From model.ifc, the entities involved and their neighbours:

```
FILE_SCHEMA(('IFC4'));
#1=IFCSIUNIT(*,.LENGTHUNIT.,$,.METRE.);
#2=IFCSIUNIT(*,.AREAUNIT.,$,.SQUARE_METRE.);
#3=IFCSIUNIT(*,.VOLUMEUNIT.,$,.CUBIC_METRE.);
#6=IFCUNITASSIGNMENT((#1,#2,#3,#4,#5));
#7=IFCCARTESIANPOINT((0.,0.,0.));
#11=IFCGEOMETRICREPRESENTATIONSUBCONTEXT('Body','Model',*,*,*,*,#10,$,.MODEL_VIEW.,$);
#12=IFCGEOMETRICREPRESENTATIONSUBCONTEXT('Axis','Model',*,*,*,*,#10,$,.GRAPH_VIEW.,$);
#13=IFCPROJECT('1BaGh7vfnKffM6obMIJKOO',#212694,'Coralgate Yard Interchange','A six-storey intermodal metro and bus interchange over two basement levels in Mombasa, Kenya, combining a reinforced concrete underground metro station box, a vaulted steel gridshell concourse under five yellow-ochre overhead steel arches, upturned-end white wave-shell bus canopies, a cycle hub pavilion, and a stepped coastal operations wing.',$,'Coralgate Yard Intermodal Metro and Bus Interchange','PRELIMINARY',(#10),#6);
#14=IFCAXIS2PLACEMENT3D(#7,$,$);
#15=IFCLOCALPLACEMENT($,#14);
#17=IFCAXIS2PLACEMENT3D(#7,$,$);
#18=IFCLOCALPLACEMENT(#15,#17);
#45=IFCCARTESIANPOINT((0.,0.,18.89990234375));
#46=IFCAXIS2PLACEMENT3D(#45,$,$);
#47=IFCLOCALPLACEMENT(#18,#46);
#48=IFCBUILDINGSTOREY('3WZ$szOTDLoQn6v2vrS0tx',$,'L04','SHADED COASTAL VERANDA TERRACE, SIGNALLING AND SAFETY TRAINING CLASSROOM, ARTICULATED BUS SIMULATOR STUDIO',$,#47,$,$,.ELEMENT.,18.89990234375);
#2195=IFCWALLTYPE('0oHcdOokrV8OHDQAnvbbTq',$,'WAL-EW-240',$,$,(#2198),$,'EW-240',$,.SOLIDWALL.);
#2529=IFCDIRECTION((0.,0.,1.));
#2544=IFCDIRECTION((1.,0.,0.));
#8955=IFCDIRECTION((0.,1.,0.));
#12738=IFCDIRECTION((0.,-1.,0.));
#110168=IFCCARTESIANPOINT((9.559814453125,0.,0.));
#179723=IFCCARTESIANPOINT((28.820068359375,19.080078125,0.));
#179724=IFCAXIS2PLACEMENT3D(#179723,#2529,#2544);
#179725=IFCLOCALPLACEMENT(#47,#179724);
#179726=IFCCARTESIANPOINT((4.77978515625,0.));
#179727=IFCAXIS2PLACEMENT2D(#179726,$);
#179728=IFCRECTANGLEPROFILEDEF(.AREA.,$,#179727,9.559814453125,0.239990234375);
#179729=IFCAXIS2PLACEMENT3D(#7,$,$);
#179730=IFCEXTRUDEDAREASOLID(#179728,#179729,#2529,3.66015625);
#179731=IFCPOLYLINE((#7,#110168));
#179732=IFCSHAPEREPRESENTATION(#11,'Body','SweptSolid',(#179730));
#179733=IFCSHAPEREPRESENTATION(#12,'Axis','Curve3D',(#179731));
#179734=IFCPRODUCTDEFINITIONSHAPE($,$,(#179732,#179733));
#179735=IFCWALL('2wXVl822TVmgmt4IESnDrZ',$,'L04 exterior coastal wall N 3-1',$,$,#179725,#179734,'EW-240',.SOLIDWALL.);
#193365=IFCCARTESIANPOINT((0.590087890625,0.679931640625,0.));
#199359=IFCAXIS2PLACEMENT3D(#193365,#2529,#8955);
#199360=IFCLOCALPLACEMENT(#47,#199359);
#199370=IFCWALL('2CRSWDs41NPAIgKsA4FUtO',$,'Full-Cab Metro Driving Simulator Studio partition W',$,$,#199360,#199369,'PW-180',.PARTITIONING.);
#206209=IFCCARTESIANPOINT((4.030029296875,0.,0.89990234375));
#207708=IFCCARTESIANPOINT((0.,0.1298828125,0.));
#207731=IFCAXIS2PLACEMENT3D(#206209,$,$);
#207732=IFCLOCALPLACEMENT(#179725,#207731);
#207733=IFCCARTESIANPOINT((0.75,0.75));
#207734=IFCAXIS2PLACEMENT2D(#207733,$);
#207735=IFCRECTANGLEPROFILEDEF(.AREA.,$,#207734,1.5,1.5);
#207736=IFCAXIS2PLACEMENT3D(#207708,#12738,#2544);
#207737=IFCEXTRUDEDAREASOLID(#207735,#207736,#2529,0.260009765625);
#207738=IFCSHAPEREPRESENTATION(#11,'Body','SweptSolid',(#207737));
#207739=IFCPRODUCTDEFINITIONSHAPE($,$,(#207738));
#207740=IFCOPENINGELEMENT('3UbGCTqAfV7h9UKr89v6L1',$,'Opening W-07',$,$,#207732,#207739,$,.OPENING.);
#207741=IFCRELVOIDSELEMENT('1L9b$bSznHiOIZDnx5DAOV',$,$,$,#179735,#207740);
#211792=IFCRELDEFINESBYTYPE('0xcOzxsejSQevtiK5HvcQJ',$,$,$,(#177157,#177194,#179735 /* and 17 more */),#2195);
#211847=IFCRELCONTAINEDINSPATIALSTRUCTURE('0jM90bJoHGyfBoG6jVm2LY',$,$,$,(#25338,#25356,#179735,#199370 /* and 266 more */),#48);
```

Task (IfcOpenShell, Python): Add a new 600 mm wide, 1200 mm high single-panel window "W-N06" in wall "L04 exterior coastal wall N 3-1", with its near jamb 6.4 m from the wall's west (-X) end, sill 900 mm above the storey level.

```python
import numpy as np
import ifcopenshell
import ifcopenshell.api.feature
import ifcopenshell.api.geometry
import ifcopenshell.api.root
import ifcopenshell.api.spatial
import ifcopenshell.geom
import ifcopenshell.util.element
import ifcopenshell.util.placement
import ifcopenshell.util.representation
import ifcopenshell.util.shape
import ifcopenshell.util.unit

model = ifcopenshell.open("model.ifc")
unit_scale = ifcopenshell.util.unit.calculate_unit_scale(model)
settings = ifcopenshell.geom.settings()


def volume(element):
    """Net volume in cubic metres, openings subtracted."""
    shape = ifcopenshell.geom.create_shape(settings, element)
    return ifcopenshell.util.shape.get_volume(shape.geometry)


wall = model.by_guid("2wXVl822TVmgmt4IESnDrZ")
storey = ifcopenshell.util.element.get_container(wall, ifc_class="IfcBuildingStorey")
context = ifcopenshell.util.representation.get_context(model, "Model", "Body", "MODEL_VIEW")
before = volume(wall)

width, height, from_end, sill = 0.6, 1.2, 6.4, 0.9  # metres

# The wall runs along its own X axis, and the end named is its -X end.
wall_shape = ifcopenshell.geom.create_shape(settings, wall)
x, y, z = ifcopenshell.util.shape.get_vertices(wall_shape.geometry).T
start = x.min() + from_end
face, thickness = float(y.min()), float(y.max() - y.min())
wall_matrix = ifcopenshell.util.placement.get_local_placement(wall.ObjectPlacement)
level = ifcopenshell.util.placement.get_local_placement(storey.ObjectPlacement)[2, 3]


def in_wall(x, y):
    """Placement at x, y metres in the wall's axes, at sill height."""
    matrix = wall_matrix.copy()
    matrix[:, 3] = wall_matrix @ np.array([x / unit_scale, y / unit_scale, 0.0, 1.0])
    matrix[2, 3] = level + sill / unit_scale
    return matrix


# Opening: a box that overshoots both wall faces by 50 mm.
opening = ifcopenshell.api.root.create_entity(model, ifc_class="IfcOpeningElement", predefined_type="OPENING")
box = ifcopenshell.api.geometry.add_wall_representation(
    model, context=context, length=width, height=height, thickness=thickness + 0.1
)
ifcopenshell.api.geometry.assign_representation(model, product=opening, representation=box)
ifcopenshell.api.geometry.edit_object_placement(model, product=opening, matrix=in_wall(start, face - 0.05), is_si=False)
ifcopenshell.api.feature.add_feature(model, feature=opening, element=wall)

window = ifcopenshell.api.root.create_entity(model, ifc_class="IfcWindow", name="W-N06", predefined_type="WINDOW")
window.OverallWidth, window.OverallHeight = width / unit_scale, height / unit_scale
window.PartitioningType = "SINGLE_PANEL"
body = ifcopenshell.api.geometry.add_window_representation(
    model,
    context=context,
    overall_width=window.OverallWidth,
    overall_height=window.OverallHeight,
    partition_type="SINGLE_PANEL",
)
ifcopenshell.api.geometry.assign_representation(model, product=window, representation=body)
ifcopenshell.api.spatial.assign_container(model, products=[window], relating_structure=storey)
ifcopenshell.api.feature.add_filling(model, opening=opening, element=window)

# Centre the window in the wall's thickness.
ifcopenshell.api.geometry.edit_object_placement(model, product=window, matrix=in_wall(start, face), is_si=False)
window_shape = ifcopenshell.geom.create_shape(settings, window)
depth = ifcopenshell.util.shape.get_vertices(window_shape.geometry)[:, 1]
offset = face + thickness / 2 - (depth.min() + depth.max()) / 2
ifcopenshell.api.geometry.edit_object_placement(model, product=window, matrix=in_wall(start, offset), is_si=False)

after = volume(wall)

print(f"wall volume {before:.3f} -> {after:.3f} m3")

model.write("model_rev.ifc")
```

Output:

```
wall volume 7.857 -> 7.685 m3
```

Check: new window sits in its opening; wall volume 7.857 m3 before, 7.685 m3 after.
